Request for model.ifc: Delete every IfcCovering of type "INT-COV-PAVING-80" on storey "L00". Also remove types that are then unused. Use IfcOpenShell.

First a look at what the model holds.

```python
import ifcopenshell
import ifcopenshell.util.element

model = ifcopenshell.open("model.ifc")
print(model.schema)
storey = next(s for s in model.by_type("IfcBuildingStorey") if s.Name == "L00")
coverings = [e for e in ifcopenshell.util.element.get_decomposition(storey) if e.is_a("IfcCovering")]
seen = {}
for e in coverings:
    element_type = ifcopenshell.util.element.get_type(e)
    name = element_type.Name if element_type not in (None, e) else None
    seen[name] = seen.get(name, 0) + 1
for name, count in sorted(seen.items(), key=str):
    print(count, "x", name)
```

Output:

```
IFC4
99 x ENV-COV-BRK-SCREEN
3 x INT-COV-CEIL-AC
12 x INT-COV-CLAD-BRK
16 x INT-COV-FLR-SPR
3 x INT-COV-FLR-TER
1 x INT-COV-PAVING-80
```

```python
import ifcopenshell
import ifcopenshell.api.root
import ifcopenshell.util.element

model = ifcopenshell.open("model.ifc")

storey = next(s for s in model.by_type("IfcBuildingStorey") if s.Name == "L00")
coverings = [e for e in ifcopenshell.util.element.get_decomposition(storey) if e.is_a("IfcCovering")]
targets = [e for e in coverings if (t := ifcopenshell.util.element.get_type(e)) not in (None, e) and t.Name == "INT-COV-PAVING-80"]
types = {ifcopenshell.util.element.get_type(e) for e in targets} - {None, *targets}

for e in targets:
    ifcopenshell.api.root.remove_product(model, product=e)
print(len(targets), "removed")

unused = [t for t in types if not ifcopenshell.util.element.get_types(t)]
for t in unused:
    ifcopenshell.api.root.remove_product(model, product=t)
print(len(unused), "unused types removed")

model.write("model_v2.ifc")
```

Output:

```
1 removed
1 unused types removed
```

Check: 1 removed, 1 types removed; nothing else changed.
